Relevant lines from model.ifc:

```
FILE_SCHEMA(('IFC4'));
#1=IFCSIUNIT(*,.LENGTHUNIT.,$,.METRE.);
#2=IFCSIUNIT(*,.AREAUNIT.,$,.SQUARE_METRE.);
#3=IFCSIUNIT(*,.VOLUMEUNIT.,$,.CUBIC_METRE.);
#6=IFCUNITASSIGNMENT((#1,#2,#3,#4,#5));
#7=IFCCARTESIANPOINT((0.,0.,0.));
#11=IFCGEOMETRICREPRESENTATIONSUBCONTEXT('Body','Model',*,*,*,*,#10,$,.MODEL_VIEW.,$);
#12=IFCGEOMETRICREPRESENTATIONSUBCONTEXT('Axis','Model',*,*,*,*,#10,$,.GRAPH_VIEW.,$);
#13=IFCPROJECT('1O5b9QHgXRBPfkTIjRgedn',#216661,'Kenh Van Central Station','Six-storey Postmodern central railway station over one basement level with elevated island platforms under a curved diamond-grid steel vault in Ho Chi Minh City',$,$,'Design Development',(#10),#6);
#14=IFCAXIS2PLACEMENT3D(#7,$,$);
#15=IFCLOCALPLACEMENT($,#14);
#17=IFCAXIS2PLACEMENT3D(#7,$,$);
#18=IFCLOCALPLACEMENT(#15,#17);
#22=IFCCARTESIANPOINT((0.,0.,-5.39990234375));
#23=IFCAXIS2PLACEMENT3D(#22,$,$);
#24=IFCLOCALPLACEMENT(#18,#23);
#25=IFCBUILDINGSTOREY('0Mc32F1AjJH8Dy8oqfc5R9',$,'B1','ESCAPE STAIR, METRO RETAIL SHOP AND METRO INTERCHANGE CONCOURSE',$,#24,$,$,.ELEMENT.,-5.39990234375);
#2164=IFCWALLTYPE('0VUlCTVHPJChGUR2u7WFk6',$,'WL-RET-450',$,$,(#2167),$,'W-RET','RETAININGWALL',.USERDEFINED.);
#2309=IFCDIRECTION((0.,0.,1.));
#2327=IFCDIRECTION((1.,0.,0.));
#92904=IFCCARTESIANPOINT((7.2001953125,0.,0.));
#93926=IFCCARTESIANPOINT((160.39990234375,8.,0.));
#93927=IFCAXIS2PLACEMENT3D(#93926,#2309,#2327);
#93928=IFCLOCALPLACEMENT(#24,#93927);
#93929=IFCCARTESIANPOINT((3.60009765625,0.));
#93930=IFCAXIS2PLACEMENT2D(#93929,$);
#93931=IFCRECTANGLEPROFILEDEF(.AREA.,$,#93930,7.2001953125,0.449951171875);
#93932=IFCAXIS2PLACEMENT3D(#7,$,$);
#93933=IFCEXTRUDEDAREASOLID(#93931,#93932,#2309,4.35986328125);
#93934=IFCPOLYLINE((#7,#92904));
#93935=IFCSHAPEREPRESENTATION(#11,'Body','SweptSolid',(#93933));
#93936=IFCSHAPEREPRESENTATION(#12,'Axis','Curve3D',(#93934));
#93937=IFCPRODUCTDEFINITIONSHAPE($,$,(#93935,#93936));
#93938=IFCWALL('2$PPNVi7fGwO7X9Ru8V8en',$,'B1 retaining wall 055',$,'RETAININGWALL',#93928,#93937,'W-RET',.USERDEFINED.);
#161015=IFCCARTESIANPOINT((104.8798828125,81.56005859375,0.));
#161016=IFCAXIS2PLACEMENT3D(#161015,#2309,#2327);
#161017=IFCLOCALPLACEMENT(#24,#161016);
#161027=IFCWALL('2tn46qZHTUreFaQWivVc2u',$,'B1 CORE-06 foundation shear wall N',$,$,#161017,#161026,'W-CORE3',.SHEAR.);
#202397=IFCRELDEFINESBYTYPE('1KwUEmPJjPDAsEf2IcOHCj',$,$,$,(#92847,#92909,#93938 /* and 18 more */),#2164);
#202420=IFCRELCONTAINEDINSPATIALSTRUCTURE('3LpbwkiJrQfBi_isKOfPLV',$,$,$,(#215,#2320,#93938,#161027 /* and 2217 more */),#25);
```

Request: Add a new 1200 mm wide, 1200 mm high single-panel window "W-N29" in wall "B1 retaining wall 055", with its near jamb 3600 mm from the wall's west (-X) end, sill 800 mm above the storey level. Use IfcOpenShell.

```python
import numpy as np
import ifcopenshell
import ifcopenshell.api.feature
import ifcopenshell.api.geometry
import ifcopenshell.api.root
import ifcopenshell.api.spatial
import ifcopenshell.geom
import ifcopenshell.util.element
import ifcopenshell.util.placement
import ifcopenshell.util.representation
import ifcopenshell.util.shape
import ifcopenshell.util.unit

model = ifcopenshell.open("model.ifc")
unit_scale = ifcopenshell.util.unit.calculate_unit_scale(model)
settings = ifcopenshell.geom.settings()


def volume(element):
    """Net volume in cubic metres, openings subtracted."""
    shape = ifcopenshell.geom.create_shape(settings, element)
    return ifcopenshell.util.shape.get_volume(shape.geometry)


wall = model.by_guid("2$PPNVi7fGwO7X9Ru8V8en")
storey = ifcopenshell.util.element.get_container(wall, ifc_class="IfcBuildingStorey")
context = ifcopenshell.util.representation.get_context(model, "Model", "Body", "MODEL_VIEW")
before = volume(wall)

width, height, from_end, sill = 1.2, 1.2, 3.6, 0.8  # metres

# The wall runs along its own X axis, and the end named is its -X end.
wall_shape = ifcopenshell.geom.create_shape(settings, wall)
x, y, z = ifcopenshell.util.shape.get_vertices(wall_shape.geometry).T
start = x.min() + from_end
face, thickness = float(y.min()), float(y.max() - y.min())
wall_matrix = ifcopenshell.util.placement.get_local_placement(wall.ObjectPlacement)
level = ifcopenshell.util.placement.get_local_placement(storey.ObjectPlacement)[2, 3]


def in_wall(x, y):
    """Placement at x, y metres in the wall's axes, at sill height."""
    matrix = wall_matrix.copy()
    matrix[:, 3] = wall_matrix @ np.array([x / unit_scale, y / unit_scale, 0.0, 1.0])
    matrix[2, 3] = level + sill / unit_scale
    return matrix


# Opening: a box that overshoots both wall faces by 50 mm.
opening = ifcopenshell.api.root.create_entity(model, ifc_class="IfcOpeningElement", predefined_type="OPENING")
box = ifcopenshell.api.geometry.add_wall_representation(
    model, context=context, length=width, height=height, thickness=thickness + 0.1
)
ifcopenshell.api.geometry.assign_representation(model, product=opening, representation=box)
ifcopenshell.api.geometry.edit_object_placement(model, product=opening, matrix=in_wall(start, face - 0.05), is_si=False)
ifcopenshell.api.feature.add_feature(model, feature=opening, element=wall)

window = ifcopenshell.api.root.create_entity(model, ifc_class="IfcWindow", name="W-N29", predefined_type="WINDOW")
window.OverallWidth, window.OverallHeight = width / unit_scale, height / unit_scale
window.PartitioningType = "SINGLE_PANEL"
body = ifcopenshell.api.geometry.add_window_representation(
    model,
    context=context,
    overall_width=window.OverallWidth,
    overall_height=window.OverallHeight,
    partition_type="SINGLE_PANEL",
)
ifcopenshell.api.geometry.assign_representation(model, product=window, representation=body)
ifcopenshell.api.spatial.assign_container(model, products=[window], relating_structure=storey)
ifcopenshell.api.feature.add_filling(model, opening=opening, element=window)

# Centre the window in the wall's thickness.
ifcopenshell.api.geometry.edit_object_placement(model, product=window, matrix=in_wall(start, face), is_si=False)
window_shape = ifcopenshell.geom.create_shape(settings, window)
depth = ifcopenshell.util.shape.get_vertices(window_shape.geometry)[:, 1]
offset = face + thickness / 2 - (depth.min() + depth.max()) / 2
ifcopenshell.api.geometry.edit_object_placement(model, product=window, matrix=in_wall(start, offset), is_si=False)

after = volume(wall)

print(f"wall volume {before:.3f} -> {after:.3f} m3")

model.write("model-out.ifc")
```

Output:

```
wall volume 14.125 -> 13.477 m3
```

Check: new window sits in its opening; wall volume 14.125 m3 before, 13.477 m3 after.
